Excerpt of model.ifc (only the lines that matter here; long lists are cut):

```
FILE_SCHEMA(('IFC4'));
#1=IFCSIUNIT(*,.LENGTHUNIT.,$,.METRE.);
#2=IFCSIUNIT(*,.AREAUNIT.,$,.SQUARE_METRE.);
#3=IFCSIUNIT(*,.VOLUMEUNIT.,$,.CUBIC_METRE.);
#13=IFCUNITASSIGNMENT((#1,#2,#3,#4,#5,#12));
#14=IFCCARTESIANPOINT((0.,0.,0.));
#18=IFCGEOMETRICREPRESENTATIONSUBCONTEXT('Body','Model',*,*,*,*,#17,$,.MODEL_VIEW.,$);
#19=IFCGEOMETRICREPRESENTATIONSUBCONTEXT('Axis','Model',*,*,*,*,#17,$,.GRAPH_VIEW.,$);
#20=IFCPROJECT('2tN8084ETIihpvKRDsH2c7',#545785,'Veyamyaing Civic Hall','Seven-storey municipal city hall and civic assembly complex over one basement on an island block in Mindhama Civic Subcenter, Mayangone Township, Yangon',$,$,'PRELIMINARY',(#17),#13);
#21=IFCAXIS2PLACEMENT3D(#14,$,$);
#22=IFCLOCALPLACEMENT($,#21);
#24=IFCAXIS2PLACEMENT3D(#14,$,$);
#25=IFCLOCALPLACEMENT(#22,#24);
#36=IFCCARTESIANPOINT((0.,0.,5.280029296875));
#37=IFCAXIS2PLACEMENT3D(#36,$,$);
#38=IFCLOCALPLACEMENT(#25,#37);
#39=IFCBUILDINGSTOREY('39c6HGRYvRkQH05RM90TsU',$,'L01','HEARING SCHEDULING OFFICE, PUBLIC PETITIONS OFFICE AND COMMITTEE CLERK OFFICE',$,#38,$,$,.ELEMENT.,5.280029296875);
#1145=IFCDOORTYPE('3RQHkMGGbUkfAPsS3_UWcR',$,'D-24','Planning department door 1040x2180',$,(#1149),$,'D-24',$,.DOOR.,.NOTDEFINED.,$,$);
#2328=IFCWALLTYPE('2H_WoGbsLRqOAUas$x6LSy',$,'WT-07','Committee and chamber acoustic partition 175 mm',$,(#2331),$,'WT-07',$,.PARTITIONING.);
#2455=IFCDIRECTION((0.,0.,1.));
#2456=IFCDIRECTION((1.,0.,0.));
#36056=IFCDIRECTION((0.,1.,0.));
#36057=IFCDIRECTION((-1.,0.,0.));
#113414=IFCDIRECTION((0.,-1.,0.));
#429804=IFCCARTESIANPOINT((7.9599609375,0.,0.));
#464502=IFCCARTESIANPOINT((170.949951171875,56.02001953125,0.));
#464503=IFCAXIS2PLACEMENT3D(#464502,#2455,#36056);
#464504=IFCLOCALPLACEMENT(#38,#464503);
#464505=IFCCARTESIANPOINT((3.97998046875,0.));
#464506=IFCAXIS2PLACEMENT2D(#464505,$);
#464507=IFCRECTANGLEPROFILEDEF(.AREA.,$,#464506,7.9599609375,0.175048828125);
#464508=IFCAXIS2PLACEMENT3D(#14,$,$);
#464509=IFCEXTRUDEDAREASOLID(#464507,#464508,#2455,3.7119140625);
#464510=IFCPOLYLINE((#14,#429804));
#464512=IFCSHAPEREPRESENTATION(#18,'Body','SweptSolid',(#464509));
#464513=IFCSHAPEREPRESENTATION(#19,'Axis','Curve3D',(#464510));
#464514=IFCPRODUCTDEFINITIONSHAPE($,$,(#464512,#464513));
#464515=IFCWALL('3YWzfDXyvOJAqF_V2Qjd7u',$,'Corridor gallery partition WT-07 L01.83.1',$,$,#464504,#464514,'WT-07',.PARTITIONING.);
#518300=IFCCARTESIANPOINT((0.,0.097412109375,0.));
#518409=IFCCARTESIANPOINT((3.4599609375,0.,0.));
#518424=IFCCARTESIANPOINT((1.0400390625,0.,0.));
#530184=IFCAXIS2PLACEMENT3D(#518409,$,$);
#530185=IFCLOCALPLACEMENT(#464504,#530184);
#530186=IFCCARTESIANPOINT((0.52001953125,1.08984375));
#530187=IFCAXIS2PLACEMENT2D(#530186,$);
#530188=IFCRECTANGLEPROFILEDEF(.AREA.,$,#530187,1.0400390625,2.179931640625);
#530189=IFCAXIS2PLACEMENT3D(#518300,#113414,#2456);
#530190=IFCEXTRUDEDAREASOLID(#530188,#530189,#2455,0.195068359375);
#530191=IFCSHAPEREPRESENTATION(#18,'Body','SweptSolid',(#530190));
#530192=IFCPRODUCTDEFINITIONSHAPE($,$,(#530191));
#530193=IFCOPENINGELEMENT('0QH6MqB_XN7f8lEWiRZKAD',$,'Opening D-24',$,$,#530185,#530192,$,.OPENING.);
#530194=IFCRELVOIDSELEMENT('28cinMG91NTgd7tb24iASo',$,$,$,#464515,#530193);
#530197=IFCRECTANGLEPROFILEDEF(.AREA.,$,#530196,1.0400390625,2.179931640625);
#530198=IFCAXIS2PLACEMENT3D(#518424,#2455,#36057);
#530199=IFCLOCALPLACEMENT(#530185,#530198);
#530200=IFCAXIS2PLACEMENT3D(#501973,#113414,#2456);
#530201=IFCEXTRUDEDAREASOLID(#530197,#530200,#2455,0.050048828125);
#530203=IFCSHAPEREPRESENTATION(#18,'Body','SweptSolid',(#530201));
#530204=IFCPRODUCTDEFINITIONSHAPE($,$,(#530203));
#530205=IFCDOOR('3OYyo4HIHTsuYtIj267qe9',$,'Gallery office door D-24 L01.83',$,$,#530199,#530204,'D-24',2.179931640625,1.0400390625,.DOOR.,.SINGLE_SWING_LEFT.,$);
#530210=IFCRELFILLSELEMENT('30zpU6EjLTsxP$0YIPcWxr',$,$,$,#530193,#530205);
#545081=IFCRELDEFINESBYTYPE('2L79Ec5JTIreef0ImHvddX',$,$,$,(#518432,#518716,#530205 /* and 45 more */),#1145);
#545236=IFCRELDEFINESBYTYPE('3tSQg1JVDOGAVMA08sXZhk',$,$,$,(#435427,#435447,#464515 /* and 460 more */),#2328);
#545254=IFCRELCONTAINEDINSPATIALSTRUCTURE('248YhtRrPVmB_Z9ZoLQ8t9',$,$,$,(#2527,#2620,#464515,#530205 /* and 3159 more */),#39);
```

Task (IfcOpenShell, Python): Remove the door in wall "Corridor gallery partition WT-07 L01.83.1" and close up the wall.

```python
import ifcopenshell
import ifcopenshell.api.feature
import ifcopenshell.api.root
import ifcopenshell.geom
import ifcopenshell.util.shape

model = ifcopenshell.open("model.ifc")
settings = ifcopenshell.geom.settings()


def volume(element):
    """Net volume in cubic metres, openings subtracted."""
    shape = ifcopenshell.geom.create_shape(settings, element)
    return ifcopenshell.util.shape.get_volume(shape.geometry)


door = model.by_id(530205)
opening = door.FillsVoids[0].RelatingOpeningElement
wall = opening.VoidsElements[0].RelatingBuildingElement
before = volume(wall)

ifcopenshell.api.root.remove_product(model, product=door)
ifcopenshell.api.feature.remove_feature(model, feature=opening)

after = volume(wall)

print(f"wall volume {before:.3f} -> {after:.3f} m3")

model.write("model_rev.ifc")
```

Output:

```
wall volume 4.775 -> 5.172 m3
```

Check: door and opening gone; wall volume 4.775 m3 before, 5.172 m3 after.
